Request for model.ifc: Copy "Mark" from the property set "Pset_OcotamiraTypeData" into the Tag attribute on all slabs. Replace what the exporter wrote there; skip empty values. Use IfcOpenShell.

First a look at what the model holds.

```python
import ifcopenshell
import ifcopenshell.util.element

model = ifcopenshell.open("model.ifc")
print(model.schema)
slabs = model.by_type("IfcSlab")
print(len(slabs), "slabs")
for e in slabs[:8]:
    source = ifcopenshell.util.element.get_pset(e, "Pset_OcotamiraTypeData", "Mark")
    target = e.Tag
    print(e.id(), repr(source), repr(target), sep=" | ")
```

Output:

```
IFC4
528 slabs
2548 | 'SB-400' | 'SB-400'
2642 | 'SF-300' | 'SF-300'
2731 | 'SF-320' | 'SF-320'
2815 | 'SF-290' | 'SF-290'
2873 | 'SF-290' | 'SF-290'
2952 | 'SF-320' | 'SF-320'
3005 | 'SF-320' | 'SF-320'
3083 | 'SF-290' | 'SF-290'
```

```python
import ifcopenshell
import ifcopenshell.util.element

model = ifcopenshell.open("model.ifc")

count = 0
for e in model.by_type("IfcSlab"):
    value = ifcopenshell.util.element.get_pset(e, "Pset_OcotamiraTypeData", "Mark")
    current = e.Tag
    if not value or not value.strip() or current == value:
        continue
    e.Tag = value
    count += 1

print(count, "slabs updated")

model.write("model_updated.ifc")
```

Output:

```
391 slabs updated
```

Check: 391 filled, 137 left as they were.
